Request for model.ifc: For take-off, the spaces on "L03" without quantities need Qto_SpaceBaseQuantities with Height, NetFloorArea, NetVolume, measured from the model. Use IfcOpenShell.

First a look at what the model holds.

```python
import ifcopenshell
import ifcopenshell.util.element
import ifcopenshell.util.unit

model = ifcopenshell.open("model.ifc")
print(model.schema)
for unit_type in ("LENGTHUNIT", "AREAUNIT", "VOLUMEUNIT"):
    print(unit_type, ifcopenshell.util.unit.calculate_unit_scale(model, unit_type))
storey = next(s for s in model.by_type("IfcBuildingStorey") if s.Name == "L03")
spaces = [e for e in ifcopenshell.util.element.get_decomposition(storey) if e.is_a("IfcSpace")]
for e in sorted(spaces, key=lambda e: e.id()):
    print(e.id(), e.is_a(), e.Name, list(ifcopenshell.util.element.get_psets(e, qtos_only=True)), sep=" | ")
```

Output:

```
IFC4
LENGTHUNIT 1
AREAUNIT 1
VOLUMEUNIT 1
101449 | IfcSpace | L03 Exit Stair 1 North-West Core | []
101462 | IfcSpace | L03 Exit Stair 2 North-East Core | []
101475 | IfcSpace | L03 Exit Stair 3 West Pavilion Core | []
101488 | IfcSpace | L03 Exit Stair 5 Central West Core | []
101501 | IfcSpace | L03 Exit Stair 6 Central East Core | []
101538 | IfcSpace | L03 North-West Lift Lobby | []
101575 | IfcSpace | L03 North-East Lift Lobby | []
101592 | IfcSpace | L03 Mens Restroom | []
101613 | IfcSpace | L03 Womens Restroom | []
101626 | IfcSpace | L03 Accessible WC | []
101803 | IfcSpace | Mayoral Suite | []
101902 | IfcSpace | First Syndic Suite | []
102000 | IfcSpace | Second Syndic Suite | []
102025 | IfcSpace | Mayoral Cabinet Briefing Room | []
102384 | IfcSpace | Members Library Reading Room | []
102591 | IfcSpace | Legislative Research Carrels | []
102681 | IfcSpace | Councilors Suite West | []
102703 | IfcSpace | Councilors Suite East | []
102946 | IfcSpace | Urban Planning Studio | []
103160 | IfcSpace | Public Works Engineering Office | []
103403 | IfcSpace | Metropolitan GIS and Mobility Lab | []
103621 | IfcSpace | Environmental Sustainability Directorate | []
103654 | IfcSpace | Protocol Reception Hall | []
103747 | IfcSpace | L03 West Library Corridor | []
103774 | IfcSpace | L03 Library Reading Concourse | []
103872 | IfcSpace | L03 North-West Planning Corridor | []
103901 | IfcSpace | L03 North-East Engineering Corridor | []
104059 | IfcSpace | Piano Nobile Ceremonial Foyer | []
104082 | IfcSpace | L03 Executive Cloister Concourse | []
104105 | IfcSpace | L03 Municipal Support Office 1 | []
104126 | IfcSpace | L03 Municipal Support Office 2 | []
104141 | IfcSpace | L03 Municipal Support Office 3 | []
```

```python
import ifcopenshell
import ifcopenshell.api.pset
import ifcopenshell.geom
import ifcopenshell.util.element
import ifcopenshell.util.shape
import ifcopenshell.util.unit

model = ifcopenshell.open("model.ifc")
unit_scale = ifcopenshell.util.unit.calculate_unit_scale(model)
area_scale = ifcopenshell.util.unit.calculate_unit_scale(model, "AREAUNIT")
volume_scale = ifcopenshell.util.unit.calculate_unit_scale(model, "VOLUMEUNIT")
settings = ifcopenshell.geom.settings()

storey = next(s for s in model.by_type("IfcBuildingStorey") if s.Name == "L03")
spaces = [e for e in ifcopenshell.util.element.get_decomposition(storey) if e.is_a("IfcSpace")]

for e in sorted(spaces, key=lambda e: e.id()):
    if ifcopenshell.util.element.get_psets(e, qtos_only=True, should_inherit=False):
        continue
    # Geometry comes back in metres, in the element's own axes.
    shape = ifcopenshell.geom.create_shape(settings, e)
    values = {
        "Height": ifcopenshell.util.shape.get_z(shape.geometry) / unit_scale,
        "NetFloorArea": ifcopenshell.util.shape.get_footprint_area(shape.geometry) / area_scale,
        "NetVolume": ifcopenshell.util.shape.get_volume(shape.geometry) / volume_scale,
    }
    qto = ifcopenshell.api.pset.add_qto(model, product=e, name="Qto_SpaceBaseQuantities")
    ifcopenshell.api.pset.edit_qto(model, qto=qto, properties=values)
    print(e.id(), {k: round(v, 3) for k, v in values.items()})

model.write("model_rev.ifc")
```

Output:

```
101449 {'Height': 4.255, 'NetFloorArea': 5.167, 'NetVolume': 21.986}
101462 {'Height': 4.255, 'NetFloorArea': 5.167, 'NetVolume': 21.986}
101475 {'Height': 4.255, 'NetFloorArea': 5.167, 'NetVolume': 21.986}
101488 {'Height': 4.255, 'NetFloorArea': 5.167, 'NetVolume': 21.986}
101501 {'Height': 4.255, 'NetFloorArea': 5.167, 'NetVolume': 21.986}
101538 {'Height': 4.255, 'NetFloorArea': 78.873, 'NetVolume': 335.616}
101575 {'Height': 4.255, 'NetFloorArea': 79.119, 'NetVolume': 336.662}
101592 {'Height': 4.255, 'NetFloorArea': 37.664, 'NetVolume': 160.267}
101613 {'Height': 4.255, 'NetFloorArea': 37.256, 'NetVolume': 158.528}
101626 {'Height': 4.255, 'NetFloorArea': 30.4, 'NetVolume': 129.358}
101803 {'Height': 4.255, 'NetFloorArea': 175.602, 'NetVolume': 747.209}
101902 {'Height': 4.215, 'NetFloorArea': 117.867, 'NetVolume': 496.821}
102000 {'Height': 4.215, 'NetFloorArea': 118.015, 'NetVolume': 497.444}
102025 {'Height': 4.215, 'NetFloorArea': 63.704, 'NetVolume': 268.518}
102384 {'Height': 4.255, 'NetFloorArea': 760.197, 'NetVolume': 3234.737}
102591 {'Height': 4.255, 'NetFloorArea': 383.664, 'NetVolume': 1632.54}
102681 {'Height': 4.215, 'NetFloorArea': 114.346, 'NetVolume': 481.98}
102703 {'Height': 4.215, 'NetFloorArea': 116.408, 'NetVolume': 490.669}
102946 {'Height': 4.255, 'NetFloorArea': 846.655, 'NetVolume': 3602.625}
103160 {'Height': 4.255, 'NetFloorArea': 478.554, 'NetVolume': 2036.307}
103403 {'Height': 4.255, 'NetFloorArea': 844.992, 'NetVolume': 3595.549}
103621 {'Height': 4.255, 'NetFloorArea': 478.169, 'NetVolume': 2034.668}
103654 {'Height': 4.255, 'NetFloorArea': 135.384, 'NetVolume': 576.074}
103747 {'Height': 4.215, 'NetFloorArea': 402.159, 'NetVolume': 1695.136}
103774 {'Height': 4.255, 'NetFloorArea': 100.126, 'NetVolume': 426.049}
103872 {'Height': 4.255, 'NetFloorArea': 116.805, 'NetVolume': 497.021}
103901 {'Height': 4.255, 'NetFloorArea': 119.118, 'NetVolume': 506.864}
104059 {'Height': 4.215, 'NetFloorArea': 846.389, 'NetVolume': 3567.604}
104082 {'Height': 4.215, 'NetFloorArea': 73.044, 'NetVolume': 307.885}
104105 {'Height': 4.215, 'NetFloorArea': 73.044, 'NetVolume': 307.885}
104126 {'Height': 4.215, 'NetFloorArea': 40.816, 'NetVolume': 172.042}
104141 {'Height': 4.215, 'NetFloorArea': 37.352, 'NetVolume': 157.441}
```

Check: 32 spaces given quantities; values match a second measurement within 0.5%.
